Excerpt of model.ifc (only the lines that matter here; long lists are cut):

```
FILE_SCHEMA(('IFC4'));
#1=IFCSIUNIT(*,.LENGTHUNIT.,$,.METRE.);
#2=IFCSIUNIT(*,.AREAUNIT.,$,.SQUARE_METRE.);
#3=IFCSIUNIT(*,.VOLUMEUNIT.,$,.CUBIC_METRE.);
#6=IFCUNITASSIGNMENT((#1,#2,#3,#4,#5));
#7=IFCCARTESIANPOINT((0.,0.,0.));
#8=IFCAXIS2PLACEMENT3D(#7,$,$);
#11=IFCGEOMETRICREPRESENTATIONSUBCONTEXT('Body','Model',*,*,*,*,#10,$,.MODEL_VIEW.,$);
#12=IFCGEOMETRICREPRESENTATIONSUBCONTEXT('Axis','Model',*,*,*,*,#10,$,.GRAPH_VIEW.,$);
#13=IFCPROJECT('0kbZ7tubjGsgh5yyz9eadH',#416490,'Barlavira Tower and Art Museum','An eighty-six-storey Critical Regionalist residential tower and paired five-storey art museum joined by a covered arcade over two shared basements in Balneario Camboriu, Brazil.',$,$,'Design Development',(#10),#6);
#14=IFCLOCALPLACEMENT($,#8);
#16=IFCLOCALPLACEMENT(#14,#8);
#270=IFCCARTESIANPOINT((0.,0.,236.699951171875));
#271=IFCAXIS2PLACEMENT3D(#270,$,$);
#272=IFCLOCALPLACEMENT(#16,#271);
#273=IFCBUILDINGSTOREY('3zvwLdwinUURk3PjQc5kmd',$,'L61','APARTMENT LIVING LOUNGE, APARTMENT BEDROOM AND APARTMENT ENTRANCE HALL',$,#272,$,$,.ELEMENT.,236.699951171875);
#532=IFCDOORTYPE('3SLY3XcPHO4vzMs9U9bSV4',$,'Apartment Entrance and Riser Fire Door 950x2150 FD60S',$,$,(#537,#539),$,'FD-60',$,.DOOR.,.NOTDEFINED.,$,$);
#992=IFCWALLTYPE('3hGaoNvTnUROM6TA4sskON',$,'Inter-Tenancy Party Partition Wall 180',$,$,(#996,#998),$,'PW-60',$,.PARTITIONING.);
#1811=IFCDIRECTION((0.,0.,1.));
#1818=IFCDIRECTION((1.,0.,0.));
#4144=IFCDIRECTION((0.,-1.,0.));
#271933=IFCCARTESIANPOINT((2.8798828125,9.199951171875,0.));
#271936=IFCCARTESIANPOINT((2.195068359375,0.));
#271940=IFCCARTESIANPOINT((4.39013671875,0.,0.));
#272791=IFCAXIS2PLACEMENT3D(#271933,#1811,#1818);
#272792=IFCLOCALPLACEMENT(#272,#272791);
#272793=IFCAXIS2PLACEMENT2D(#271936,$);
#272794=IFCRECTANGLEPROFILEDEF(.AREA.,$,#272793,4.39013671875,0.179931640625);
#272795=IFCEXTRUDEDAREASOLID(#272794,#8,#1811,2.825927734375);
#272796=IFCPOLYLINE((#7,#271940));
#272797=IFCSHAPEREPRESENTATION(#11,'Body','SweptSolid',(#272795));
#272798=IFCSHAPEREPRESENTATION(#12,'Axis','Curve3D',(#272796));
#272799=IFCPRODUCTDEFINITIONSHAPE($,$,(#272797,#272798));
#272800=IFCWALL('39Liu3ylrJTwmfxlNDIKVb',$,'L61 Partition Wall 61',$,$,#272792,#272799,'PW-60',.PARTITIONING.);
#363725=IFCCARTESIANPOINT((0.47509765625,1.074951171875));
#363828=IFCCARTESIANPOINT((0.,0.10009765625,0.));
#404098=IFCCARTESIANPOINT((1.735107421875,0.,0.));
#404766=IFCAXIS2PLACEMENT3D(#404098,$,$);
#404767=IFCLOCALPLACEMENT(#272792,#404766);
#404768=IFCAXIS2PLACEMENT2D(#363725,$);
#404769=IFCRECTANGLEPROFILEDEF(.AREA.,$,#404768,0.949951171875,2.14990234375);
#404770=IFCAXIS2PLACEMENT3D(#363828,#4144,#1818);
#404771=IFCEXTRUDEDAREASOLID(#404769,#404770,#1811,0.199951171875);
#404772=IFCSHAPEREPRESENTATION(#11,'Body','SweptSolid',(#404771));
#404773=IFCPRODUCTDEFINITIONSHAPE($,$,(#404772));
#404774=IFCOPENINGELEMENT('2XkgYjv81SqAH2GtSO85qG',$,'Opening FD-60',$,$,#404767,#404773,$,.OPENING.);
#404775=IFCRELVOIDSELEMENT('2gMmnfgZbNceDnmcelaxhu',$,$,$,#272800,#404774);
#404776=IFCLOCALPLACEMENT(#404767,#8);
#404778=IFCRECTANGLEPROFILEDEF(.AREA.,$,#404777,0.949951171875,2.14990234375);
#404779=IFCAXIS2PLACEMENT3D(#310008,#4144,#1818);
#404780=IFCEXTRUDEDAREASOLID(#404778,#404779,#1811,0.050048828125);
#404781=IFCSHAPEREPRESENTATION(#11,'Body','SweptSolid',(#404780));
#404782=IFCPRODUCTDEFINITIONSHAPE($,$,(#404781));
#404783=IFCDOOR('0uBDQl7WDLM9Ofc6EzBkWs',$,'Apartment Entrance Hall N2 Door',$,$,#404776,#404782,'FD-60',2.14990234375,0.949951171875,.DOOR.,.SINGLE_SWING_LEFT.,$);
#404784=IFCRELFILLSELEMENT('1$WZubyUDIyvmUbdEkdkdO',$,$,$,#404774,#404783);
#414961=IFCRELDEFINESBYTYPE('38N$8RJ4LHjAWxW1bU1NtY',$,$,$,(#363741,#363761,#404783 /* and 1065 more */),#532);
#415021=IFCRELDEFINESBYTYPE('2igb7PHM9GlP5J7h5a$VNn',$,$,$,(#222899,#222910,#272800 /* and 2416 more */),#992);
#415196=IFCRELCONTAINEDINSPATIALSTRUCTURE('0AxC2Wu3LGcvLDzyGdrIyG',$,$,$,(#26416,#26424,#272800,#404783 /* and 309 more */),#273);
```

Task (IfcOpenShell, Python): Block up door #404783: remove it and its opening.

```python
import ifcopenshell
import ifcopenshell.api.feature
import ifcopenshell.api.root
import ifcopenshell.geom
import ifcopenshell.util.shape

model = ifcopenshell.open("model.ifc")
settings = ifcopenshell.geom.settings()


def volume(element):
    """Net volume in cubic metres, openings subtracted."""
    shape = ifcopenshell.geom.create_shape(settings, element)
    return ifcopenshell.util.shape.get_volume(shape.geometry)


door = model.by_guid("0uBDQl7WDLM9Ofc6EzBkWs")
opening = door.FillsVoids[0].RelatingOpeningElement
wall = opening.VoidsElements[0].RelatingBuildingElement
before = volume(wall)

ifcopenshell.api.root.remove_product(model, product=door)
ifcopenshell.api.feature.remove_feature(model, feature=opening)

after = volume(wall)

print(f"wall volume {before:.3f} -> {after:.3f} m3")

model.write("model_edited.ifc")
```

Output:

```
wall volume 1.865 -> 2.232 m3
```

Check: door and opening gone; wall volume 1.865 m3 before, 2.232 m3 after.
